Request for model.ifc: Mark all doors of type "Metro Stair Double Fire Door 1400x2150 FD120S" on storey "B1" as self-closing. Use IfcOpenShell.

First a look at what the model holds.

```python
import ifcopenshell
import ifcopenshell.util.element

model = ifcopenshell.open("model.ifc")
print(model.schema)
storey = next(s for s in model.by_type("IfcBuildingStorey") if s.Name == "B1")
doors = [e for e in ifcopenshell.util.element.get_decomposition(storey) if e.is_a("IfcDoor")]
seen = {}
for e in doors:
    element_type = ifcopenshell.util.element.get_type(e)
    key = (element_type.Name if element_type != e and element_type else None, ifcopenshell.util.element.get_pset(e, "Pset_DoorCommon", "SelfClosing"))
    seen[key] = seen.get(key, 0) + 1
for (name, value), count in sorted(seen.items(), key=str):
    print(count, "x", name, "|", value)
```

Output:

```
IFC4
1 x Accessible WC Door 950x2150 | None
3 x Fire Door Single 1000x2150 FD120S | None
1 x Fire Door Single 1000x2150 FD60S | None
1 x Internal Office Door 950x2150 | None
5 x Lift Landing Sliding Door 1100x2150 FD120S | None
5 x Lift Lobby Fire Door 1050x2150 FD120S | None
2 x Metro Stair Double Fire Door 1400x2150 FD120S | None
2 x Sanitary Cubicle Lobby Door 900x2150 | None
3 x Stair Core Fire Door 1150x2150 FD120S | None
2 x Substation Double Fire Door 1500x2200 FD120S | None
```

```python
import ifcopenshell
import ifcopenshell.api.pset
import ifcopenshell.util.element

model = ifcopenshell.open("model.ifc")

storey = next(s for s in model.by_type("IfcBuildingStorey") if s.Name == "B1")
doors = [e for e in ifcopenshell.util.element.get_decomposition(storey) if e.is_a("IfcDoor")]

count = 0
for e in doors:
    element_type = ifcopenshell.util.element.get_type(e)
    if element_type in (None, e) or element_type.Name != "Metro Stair Double Fire Door 1400x2150 FD120S":
        continue
    # add_pset returns the element's existing set when there is one.
    pset = ifcopenshell.api.pset.add_pset(model, product=e, name="Pset_DoorCommon")
    ifcopenshell.api.pset.edit_pset(model, pset=pset, properties={"SelfClosing": True})
    count += 1

print(count, "doors updated")

model.write("model_updated.ifc")
```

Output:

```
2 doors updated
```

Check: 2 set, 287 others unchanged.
